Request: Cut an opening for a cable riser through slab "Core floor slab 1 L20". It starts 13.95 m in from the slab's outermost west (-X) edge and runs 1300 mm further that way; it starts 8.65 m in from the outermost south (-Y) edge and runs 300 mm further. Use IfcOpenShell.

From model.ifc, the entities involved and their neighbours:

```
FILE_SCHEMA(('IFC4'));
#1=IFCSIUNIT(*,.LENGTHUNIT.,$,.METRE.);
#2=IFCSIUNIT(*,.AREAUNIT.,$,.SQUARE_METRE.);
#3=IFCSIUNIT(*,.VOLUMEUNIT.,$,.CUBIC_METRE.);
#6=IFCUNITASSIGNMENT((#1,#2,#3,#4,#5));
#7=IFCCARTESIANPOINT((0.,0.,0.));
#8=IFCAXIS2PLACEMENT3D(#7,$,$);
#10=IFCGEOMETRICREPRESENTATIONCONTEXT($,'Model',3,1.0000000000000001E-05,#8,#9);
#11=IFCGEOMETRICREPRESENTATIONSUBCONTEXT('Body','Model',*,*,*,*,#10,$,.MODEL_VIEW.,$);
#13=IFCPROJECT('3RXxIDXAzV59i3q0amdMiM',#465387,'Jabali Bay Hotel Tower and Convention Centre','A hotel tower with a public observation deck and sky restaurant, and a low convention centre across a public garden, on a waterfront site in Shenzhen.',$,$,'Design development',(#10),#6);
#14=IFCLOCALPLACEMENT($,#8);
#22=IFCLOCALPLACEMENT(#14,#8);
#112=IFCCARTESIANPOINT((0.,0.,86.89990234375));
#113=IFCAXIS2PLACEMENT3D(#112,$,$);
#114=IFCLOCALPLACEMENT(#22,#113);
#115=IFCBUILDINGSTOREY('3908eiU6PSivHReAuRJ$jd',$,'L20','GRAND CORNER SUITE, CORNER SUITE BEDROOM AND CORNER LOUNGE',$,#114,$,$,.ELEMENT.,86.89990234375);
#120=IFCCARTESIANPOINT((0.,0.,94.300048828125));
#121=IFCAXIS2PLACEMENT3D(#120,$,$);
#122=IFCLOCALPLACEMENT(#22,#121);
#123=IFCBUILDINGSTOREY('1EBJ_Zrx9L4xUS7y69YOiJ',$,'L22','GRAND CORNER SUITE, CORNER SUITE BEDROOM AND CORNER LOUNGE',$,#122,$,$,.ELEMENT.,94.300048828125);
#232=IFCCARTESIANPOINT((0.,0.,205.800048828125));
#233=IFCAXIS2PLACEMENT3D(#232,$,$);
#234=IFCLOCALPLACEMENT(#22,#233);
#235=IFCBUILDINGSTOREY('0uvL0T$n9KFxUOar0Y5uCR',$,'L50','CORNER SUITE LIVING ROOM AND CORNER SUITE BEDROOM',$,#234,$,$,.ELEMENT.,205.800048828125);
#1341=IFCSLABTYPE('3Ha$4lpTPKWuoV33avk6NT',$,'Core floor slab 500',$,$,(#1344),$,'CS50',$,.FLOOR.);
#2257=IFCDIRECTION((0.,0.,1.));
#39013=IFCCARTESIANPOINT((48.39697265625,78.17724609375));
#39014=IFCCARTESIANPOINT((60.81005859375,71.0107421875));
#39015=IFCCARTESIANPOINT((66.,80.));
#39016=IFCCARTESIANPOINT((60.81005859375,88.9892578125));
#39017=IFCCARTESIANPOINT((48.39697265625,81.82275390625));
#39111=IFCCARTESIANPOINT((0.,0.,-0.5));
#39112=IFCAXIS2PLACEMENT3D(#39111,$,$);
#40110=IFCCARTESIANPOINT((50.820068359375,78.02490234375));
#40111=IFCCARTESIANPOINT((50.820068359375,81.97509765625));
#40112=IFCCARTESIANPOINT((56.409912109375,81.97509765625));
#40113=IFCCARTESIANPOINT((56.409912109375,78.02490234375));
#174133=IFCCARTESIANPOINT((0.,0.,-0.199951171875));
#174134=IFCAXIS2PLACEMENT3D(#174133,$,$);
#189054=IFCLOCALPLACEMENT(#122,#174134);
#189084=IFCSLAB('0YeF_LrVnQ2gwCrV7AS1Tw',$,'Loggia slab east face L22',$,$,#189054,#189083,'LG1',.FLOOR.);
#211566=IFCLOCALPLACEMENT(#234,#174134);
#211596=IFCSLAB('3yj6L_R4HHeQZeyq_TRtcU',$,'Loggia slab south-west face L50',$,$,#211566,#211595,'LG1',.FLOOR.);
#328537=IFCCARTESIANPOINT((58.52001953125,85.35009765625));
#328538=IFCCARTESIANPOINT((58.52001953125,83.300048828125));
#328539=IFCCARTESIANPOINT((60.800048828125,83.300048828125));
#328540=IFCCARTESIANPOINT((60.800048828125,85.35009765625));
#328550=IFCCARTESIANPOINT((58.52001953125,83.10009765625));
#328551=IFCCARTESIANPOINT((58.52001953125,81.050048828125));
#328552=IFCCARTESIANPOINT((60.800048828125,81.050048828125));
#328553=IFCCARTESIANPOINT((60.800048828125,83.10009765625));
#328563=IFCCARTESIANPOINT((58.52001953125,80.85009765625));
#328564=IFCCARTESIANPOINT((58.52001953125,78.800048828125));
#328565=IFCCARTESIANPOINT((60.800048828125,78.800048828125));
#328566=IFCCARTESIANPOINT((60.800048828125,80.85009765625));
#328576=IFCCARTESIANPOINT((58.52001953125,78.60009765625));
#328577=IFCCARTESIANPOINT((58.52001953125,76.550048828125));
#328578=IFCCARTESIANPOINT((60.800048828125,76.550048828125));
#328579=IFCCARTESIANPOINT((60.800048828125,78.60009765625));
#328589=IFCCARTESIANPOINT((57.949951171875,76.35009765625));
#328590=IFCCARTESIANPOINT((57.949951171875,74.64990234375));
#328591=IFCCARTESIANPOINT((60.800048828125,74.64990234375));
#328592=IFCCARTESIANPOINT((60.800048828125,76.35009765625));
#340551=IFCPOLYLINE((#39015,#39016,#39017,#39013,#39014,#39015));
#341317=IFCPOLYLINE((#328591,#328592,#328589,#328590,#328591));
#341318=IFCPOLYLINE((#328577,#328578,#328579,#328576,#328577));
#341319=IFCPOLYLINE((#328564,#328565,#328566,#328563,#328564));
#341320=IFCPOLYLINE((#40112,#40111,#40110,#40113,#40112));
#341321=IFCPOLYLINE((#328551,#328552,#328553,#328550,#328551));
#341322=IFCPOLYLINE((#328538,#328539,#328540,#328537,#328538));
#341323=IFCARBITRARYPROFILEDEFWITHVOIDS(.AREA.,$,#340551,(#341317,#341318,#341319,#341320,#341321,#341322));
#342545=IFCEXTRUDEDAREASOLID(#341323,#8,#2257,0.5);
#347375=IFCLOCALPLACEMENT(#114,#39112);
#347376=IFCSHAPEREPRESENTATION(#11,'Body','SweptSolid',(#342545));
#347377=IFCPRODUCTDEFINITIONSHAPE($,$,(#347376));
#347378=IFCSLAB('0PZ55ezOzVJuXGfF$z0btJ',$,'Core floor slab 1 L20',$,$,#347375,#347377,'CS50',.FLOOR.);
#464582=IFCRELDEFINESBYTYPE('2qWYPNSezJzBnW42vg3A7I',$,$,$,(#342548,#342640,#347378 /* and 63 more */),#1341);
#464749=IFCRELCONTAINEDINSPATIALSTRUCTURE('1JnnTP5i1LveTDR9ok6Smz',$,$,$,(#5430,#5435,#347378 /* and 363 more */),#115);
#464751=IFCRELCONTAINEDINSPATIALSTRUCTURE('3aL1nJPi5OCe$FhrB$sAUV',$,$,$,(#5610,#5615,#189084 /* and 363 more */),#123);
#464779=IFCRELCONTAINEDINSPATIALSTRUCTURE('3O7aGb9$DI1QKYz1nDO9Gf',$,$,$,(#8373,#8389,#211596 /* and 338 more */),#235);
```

```python
import numpy as np
import ifcopenshell
import ifcopenshell.api.feature
import ifcopenshell.api.geometry
import ifcopenshell.api.root
import ifcopenshell.geom
import ifcopenshell.util.placement
import ifcopenshell.util.representation
import ifcopenshell.util.shape
import ifcopenshell.util.unit

model = ifcopenshell.open("model.ifc")
unit_scale = ifcopenshell.util.unit.calculate_unit_scale(model)
settings = ifcopenshell.geom.settings()


def volume(element):
    """Net volume in cubic metres, openings subtracted."""
    shape = ifcopenshell.geom.create_shape(settings, element)
    return ifcopenshell.util.shape.get_volume(shape.geometry)


slab = model.by_guid("0PZ55ezOzVJuXGfF$z0btJ")
before = volume(slab)

# Extent in the slab's own axes, in metres. The edges named are its -X and -Y sides.
slab_shape = ifcopenshell.geom.create_shape(settings, slab)
vertices = ifcopenshell.util.shape.get_vertices(slab_shape.geometry)
x_min, y_min, bottom = vertices.min(axis=0)
top = vertices[:, 2].max()

opening = ifcopenshell.api.root.create_entity(model, ifc_class="IfcOpeningElement", name="Cable riser opening", predefined_type="OPENING")
context = ifcopenshell.util.representation.get_context(model, "Model", "Body", "MODEL_VIEW")
width, depth = 1.3, 0.3
outline = [(0.0, 0.0), (width, 0.0), (width, depth), (0.0, depth), (0.0, 0.0)]
# Overshoot both faces by 50 mm so the cut is clean.
shape = ifcopenshell.api.geometry.add_slab_representation(
    model, context=context, depth=top - bottom + 0.1, polyline=outline
)
ifcopenshell.api.geometry.assign_representation(model, product=opening, representation=shape)

matrix = ifcopenshell.util.placement.get_local_placement(slab.ObjectPlacement)
matrix[:, 3] = matrix @ np.append(np.array([x_min + 13.95, y_min + 8.65, bottom - 0.05]) / unit_scale, 1.0)
ifcopenshell.api.geometry.edit_object_placement(model, product=opening, matrix=matrix, is_si=False)
ifcopenshell.api.feature.add_feature(model, feature=opening, element=slab)

after = volume(slab)

print(f"slab volume {before:.3f} -> {after:.3f} m3")

model.write("model-out.ifc")
```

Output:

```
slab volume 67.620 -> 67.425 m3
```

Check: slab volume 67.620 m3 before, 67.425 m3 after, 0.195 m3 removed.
